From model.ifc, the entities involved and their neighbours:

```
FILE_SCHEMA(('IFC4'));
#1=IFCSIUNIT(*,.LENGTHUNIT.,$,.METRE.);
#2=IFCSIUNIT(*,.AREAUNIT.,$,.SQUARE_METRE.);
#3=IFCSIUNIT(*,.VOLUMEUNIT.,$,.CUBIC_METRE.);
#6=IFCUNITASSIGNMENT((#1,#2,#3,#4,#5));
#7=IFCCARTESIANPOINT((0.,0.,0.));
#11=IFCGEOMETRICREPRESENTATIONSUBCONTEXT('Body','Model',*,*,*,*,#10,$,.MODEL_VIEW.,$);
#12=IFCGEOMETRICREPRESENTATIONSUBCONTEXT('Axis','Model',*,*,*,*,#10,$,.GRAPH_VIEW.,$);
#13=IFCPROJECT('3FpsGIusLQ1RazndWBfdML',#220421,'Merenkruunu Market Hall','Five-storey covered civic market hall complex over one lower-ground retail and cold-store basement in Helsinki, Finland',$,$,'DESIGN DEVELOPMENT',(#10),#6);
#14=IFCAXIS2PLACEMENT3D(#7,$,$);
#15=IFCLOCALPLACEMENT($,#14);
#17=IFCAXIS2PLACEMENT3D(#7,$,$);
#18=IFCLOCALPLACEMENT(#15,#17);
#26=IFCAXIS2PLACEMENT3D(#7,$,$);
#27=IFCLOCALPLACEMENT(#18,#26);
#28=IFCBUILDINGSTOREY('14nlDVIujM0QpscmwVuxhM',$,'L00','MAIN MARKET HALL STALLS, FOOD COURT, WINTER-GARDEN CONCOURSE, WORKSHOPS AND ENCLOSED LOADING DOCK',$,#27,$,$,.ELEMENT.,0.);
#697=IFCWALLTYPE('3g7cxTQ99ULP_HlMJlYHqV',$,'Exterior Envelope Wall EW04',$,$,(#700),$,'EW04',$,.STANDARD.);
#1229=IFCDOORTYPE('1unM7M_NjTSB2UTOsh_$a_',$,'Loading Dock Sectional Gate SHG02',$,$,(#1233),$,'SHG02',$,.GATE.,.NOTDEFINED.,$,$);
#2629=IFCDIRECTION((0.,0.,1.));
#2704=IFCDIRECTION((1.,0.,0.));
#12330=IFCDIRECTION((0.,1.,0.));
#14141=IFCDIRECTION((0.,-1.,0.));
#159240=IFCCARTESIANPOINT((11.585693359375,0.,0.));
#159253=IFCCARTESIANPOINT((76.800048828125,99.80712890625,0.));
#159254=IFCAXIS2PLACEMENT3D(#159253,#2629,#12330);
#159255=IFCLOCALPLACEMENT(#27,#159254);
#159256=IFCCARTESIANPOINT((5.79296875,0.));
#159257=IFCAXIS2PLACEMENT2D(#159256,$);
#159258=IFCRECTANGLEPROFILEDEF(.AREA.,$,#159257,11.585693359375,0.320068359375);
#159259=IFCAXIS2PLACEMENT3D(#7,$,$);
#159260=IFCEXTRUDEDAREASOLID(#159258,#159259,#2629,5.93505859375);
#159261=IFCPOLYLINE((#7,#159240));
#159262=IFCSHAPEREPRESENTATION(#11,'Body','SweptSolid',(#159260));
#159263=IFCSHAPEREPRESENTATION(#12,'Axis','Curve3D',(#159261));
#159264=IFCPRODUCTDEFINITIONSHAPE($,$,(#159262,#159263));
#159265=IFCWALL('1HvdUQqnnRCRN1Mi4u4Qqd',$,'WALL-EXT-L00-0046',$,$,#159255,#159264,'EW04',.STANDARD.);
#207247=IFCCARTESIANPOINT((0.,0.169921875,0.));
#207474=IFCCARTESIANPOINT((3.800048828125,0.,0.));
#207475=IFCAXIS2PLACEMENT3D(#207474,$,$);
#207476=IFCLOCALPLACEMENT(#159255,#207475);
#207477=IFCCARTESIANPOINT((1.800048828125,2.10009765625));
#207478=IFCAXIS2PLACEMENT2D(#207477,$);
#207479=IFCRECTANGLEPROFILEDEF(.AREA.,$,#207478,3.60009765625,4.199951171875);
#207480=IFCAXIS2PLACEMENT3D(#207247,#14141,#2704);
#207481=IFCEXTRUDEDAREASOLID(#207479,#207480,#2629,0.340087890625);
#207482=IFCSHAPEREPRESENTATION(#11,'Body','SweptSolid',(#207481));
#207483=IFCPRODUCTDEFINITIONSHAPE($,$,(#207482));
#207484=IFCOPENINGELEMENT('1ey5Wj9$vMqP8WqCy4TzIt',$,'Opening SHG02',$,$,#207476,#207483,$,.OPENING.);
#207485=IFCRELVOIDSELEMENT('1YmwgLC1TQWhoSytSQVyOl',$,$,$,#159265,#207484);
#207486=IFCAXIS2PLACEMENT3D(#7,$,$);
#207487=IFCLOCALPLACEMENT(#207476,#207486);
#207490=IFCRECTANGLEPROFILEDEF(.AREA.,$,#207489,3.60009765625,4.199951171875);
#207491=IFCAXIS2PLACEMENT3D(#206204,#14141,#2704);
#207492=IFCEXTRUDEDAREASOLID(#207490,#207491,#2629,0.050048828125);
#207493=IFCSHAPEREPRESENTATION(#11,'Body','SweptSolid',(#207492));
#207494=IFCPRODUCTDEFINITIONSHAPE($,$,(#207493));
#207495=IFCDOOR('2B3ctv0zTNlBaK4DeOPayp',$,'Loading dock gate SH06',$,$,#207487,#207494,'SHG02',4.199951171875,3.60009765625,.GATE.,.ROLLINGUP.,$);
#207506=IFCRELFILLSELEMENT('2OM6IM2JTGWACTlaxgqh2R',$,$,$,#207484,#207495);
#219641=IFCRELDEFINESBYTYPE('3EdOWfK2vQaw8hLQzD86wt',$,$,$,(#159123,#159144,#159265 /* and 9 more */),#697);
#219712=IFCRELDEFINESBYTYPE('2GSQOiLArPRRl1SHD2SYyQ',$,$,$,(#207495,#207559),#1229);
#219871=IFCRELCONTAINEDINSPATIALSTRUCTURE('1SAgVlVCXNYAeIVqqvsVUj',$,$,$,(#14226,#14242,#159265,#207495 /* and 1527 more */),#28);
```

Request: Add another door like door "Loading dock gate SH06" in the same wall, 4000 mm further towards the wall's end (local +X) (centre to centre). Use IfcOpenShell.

```python
import ifcopenshell
import ifcopenshell.api.feature
import ifcopenshell.api.geometry
import ifcopenshell.api.root
import ifcopenshell.geom
import ifcopenshell.util.element
import ifcopenshell.util.placement
import ifcopenshell.util.shape

model = ifcopenshell.open("model.ifc")
settings = ifcopenshell.geom.settings()


def volume(element):
    """Net volume in cubic metres, openings subtracted."""
    shape = ifcopenshell.geom.create_shape(settings, element)
    return ifcopenshell.util.shape.get_volume(shape.geometry)


door = model.by_id(207495)
opening = door.FillsVoids[0].RelatingOpeningElement
wall = opening.VoidsElements[0].RelatingBuildingElement
before = volume(wall)
shift = ifcopenshell.util.placement.get_local_placement(wall.ObjectPlacement)[:3, 0] * 4.0

# copy_class copies the void relationship, type, container and properties, but no geometry.
new_opening = ifcopenshell.api.root.copy_class(model, product=opening)
new_opening.Representation = ifcopenshell.util.element.copy_deep(
    model, opening.Representation, exclude=["IfcGeometricRepresentationContext", "IfcRepresentationMap"]
)
new_door = ifcopenshell.api.root.copy_class(model, product=door)
new_door.Representation = ifcopenshell.util.element.copy_deep(
    model, door.Representation, exclude=["IfcGeometricRepresentationContext", "IfcRepresentationMap"]
)
new_door.Tag = None
ifcopenshell.api.feature.add_filling(model, opening=new_opening, element=new_door)

for old, new in ((opening, new_opening), (door, new_door)):
    matrix = ifcopenshell.util.placement.get_local_placement(old.ObjectPlacement)
    matrix[:3, 3] += shift
    ifcopenshell.api.geometry.edit_object_placement(model, product=new, matrix=matrix, is_si=False)

after = volume(wall)

print(f"wall volume {before:.3f} -> {after:.3f} m3")

model.write("model_updated.ifc")
```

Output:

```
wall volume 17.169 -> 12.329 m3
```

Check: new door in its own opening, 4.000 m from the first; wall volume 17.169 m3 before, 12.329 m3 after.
